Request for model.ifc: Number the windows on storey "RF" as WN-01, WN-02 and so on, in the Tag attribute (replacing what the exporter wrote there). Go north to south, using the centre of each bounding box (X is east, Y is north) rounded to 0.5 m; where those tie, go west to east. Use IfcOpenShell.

First a look at what the model holds.

```python
import ifcopenshell
import ifcopenshell.util.element
import ifcopenshell.util.placement

model = ifcopenshell.open("model.ifc")
print(model.schema)
storey = next(s for s in model.by_type("IfcBuildingStorey") if s.Name == "RF")
windows = [e for e in ifcopenshell.util.element.get_decomposition(storey) if e.is_a("IfcWindow")]
for e in sorted(windows, key=lambda e: e.id()):
    origin = ifcopenshell.util.placement.get_local_placement(e.ObjectPlacement)[:3, 3]
    print(e.id(), e.Tag, e.Name, origin.round(2) + 0.0, sep=" | ")
```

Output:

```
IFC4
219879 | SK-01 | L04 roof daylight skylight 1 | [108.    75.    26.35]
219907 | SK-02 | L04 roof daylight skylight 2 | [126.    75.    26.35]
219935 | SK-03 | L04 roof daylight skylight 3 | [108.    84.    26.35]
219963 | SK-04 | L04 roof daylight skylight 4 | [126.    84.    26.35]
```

```python
import ifcopenshell
import ifcopenshell.geom
import ifcopenshell.util.element
import ifcopenshell.util.shape

model = ifcopenshell.open("model.ifc")
settings = ifcopenshell.geom.settings()
settings.set("use-world-coords", True)


def centre(element):
    shape = ifcopenshell.geom.create_shape(settings, element)
    return ifcopenshell.util.shape.get_bbox_centroid(shape.geometry)


storey = next(s for s in model.by_type("IfcBuildingStorey") if s.Name == "RF")
windows = [e for e in ifcopenshell.util.element.get_decomposition(storey) if e.is_a("IfcWindow")]

# Insertion points can sit at a corner or the storey origin, so sort by the geometry (in metres).
centres = {e: centre(e) for e in windows}
windows.sort(key=lambda e: (-round(centres[e][1] / 0.5), centres[e][0]))

for i, e in enumerate(windows, start=1):
    number = f"WN-{i:02d}"
    e.Tag = number
    print(e.id(), number)

model.write("model_rev.ifc")
```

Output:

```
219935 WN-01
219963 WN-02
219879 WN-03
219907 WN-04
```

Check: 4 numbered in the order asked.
